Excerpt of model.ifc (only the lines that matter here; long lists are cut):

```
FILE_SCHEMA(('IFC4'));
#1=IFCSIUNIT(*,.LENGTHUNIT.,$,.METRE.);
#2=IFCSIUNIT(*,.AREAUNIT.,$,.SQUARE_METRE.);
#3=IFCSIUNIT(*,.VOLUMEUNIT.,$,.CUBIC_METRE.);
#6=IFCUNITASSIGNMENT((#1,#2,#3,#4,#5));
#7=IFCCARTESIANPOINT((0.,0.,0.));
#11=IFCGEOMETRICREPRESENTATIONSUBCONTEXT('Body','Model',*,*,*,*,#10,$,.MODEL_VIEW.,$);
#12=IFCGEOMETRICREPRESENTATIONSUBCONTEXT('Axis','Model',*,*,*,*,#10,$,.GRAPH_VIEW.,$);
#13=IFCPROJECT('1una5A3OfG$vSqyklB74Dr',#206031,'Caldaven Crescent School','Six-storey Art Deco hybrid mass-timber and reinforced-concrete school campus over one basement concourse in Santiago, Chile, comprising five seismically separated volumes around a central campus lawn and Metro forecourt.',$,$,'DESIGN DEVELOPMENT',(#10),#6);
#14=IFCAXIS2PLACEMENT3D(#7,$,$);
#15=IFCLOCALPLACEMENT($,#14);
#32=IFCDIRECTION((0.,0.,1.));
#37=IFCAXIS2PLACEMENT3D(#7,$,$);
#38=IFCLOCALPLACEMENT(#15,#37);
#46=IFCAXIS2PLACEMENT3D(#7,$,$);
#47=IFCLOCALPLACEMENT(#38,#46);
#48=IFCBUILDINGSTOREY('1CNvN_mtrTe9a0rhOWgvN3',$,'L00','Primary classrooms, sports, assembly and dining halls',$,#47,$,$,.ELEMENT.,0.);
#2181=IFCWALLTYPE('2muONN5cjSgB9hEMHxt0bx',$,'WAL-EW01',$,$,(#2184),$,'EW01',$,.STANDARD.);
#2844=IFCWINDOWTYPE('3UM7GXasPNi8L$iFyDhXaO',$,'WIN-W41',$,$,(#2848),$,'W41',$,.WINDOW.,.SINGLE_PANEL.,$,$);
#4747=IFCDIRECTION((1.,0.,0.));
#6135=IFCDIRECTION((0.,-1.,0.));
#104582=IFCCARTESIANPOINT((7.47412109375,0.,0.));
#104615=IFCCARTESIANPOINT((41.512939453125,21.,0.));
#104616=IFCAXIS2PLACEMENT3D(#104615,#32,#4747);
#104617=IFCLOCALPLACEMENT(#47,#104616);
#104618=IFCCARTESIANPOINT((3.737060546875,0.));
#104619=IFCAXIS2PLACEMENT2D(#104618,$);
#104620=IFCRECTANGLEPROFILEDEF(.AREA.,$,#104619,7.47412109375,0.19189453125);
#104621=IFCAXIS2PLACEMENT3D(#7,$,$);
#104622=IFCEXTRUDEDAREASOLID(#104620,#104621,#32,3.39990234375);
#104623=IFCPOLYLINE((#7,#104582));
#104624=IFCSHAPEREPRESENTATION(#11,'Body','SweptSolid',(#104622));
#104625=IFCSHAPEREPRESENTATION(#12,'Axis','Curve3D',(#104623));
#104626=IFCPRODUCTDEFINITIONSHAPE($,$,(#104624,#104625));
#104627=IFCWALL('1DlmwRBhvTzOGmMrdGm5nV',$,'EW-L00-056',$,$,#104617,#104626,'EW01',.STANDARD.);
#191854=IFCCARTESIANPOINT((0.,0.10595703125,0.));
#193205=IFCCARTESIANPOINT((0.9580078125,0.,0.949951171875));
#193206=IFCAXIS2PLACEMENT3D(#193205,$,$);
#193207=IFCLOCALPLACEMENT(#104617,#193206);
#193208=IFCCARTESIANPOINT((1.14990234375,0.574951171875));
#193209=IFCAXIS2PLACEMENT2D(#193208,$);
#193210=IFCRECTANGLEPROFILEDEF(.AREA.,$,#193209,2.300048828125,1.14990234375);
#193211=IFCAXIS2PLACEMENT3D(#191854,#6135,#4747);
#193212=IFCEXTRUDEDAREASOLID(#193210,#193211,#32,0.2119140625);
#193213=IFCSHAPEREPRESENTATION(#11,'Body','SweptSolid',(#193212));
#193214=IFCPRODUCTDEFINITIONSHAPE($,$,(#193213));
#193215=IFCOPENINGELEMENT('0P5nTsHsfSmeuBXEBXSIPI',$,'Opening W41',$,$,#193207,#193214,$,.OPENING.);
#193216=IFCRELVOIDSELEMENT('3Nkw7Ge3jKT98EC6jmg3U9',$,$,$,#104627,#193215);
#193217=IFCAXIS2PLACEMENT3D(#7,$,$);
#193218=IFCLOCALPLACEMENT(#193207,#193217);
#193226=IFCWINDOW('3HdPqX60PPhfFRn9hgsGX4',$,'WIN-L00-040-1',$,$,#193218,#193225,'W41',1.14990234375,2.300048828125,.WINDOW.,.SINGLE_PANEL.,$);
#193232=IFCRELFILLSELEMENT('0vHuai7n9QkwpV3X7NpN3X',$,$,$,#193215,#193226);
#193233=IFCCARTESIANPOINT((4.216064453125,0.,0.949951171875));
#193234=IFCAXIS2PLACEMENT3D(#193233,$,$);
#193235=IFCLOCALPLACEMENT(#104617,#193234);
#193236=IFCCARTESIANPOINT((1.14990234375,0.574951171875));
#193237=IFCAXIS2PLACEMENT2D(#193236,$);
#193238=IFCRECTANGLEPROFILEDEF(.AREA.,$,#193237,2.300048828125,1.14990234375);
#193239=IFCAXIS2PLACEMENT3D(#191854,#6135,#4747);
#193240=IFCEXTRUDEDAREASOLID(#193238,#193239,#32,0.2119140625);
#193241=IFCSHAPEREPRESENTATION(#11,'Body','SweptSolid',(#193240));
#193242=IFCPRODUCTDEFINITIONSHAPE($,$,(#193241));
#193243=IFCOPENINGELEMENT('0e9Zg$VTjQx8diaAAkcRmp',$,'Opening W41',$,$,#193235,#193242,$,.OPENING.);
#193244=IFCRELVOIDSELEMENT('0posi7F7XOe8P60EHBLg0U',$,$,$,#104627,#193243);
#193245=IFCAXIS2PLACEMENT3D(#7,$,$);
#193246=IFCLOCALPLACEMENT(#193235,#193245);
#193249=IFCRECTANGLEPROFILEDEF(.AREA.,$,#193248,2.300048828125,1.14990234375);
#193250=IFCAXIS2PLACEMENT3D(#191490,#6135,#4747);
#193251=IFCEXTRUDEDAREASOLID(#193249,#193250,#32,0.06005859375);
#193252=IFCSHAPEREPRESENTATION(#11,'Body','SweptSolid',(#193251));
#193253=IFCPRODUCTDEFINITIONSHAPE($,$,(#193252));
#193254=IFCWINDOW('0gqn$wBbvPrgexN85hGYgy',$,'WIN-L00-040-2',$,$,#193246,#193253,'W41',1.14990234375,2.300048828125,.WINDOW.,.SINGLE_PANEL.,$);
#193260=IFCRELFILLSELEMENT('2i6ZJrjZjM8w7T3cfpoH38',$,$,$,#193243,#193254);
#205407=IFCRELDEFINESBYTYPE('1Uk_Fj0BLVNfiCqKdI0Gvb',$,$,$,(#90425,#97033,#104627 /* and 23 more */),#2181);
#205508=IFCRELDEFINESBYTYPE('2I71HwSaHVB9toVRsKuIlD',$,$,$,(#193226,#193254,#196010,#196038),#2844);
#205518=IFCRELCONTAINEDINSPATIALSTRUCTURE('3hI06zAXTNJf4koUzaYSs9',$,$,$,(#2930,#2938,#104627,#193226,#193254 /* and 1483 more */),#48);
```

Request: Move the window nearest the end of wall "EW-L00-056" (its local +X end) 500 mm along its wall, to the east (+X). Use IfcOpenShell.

```python
import ifcopenshell
import ifcopenshell.api.geometry
import ifcopenshell.util.placement

model = ifcopenshell.open("model.ifc")

window = model.by_id(193254)
opening = window.FillsVoids[0].RelatingOpeningElement
wall = opening.VoidsElements[0].RelatingBuildingElement

wall_matrix = ifcopenshell.util.placement.get_local_placement(wall.ObjectPlacement)
shift = wall_matrix[:3, 0] * 0.5
before = ifcopenshell.util.placement.get_local_placement(window.ObjectPlacement)[:3, 3].copy()

# The window is placed relative to its opening, so it follows when the opening moves.
matrix = ifcopenshell.util.placement.get_local_placement(opening.ObjectPlacement)
matrix[:3, 3] += shift
ifcopenshell.api.geometry.edit_object_placement(
    model, product=opening, matrix=matrix, is_si=False, should_transform_children=True
)

after = ifcopenshell.util.placement.get_local_placement(window.ObjectPlacement)[:3, 3]
print("window moved by", (after - before).round(3) + 0.0)

model.write("model_rev.ifc")
```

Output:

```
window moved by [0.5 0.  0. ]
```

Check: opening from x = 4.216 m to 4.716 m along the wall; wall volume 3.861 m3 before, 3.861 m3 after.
